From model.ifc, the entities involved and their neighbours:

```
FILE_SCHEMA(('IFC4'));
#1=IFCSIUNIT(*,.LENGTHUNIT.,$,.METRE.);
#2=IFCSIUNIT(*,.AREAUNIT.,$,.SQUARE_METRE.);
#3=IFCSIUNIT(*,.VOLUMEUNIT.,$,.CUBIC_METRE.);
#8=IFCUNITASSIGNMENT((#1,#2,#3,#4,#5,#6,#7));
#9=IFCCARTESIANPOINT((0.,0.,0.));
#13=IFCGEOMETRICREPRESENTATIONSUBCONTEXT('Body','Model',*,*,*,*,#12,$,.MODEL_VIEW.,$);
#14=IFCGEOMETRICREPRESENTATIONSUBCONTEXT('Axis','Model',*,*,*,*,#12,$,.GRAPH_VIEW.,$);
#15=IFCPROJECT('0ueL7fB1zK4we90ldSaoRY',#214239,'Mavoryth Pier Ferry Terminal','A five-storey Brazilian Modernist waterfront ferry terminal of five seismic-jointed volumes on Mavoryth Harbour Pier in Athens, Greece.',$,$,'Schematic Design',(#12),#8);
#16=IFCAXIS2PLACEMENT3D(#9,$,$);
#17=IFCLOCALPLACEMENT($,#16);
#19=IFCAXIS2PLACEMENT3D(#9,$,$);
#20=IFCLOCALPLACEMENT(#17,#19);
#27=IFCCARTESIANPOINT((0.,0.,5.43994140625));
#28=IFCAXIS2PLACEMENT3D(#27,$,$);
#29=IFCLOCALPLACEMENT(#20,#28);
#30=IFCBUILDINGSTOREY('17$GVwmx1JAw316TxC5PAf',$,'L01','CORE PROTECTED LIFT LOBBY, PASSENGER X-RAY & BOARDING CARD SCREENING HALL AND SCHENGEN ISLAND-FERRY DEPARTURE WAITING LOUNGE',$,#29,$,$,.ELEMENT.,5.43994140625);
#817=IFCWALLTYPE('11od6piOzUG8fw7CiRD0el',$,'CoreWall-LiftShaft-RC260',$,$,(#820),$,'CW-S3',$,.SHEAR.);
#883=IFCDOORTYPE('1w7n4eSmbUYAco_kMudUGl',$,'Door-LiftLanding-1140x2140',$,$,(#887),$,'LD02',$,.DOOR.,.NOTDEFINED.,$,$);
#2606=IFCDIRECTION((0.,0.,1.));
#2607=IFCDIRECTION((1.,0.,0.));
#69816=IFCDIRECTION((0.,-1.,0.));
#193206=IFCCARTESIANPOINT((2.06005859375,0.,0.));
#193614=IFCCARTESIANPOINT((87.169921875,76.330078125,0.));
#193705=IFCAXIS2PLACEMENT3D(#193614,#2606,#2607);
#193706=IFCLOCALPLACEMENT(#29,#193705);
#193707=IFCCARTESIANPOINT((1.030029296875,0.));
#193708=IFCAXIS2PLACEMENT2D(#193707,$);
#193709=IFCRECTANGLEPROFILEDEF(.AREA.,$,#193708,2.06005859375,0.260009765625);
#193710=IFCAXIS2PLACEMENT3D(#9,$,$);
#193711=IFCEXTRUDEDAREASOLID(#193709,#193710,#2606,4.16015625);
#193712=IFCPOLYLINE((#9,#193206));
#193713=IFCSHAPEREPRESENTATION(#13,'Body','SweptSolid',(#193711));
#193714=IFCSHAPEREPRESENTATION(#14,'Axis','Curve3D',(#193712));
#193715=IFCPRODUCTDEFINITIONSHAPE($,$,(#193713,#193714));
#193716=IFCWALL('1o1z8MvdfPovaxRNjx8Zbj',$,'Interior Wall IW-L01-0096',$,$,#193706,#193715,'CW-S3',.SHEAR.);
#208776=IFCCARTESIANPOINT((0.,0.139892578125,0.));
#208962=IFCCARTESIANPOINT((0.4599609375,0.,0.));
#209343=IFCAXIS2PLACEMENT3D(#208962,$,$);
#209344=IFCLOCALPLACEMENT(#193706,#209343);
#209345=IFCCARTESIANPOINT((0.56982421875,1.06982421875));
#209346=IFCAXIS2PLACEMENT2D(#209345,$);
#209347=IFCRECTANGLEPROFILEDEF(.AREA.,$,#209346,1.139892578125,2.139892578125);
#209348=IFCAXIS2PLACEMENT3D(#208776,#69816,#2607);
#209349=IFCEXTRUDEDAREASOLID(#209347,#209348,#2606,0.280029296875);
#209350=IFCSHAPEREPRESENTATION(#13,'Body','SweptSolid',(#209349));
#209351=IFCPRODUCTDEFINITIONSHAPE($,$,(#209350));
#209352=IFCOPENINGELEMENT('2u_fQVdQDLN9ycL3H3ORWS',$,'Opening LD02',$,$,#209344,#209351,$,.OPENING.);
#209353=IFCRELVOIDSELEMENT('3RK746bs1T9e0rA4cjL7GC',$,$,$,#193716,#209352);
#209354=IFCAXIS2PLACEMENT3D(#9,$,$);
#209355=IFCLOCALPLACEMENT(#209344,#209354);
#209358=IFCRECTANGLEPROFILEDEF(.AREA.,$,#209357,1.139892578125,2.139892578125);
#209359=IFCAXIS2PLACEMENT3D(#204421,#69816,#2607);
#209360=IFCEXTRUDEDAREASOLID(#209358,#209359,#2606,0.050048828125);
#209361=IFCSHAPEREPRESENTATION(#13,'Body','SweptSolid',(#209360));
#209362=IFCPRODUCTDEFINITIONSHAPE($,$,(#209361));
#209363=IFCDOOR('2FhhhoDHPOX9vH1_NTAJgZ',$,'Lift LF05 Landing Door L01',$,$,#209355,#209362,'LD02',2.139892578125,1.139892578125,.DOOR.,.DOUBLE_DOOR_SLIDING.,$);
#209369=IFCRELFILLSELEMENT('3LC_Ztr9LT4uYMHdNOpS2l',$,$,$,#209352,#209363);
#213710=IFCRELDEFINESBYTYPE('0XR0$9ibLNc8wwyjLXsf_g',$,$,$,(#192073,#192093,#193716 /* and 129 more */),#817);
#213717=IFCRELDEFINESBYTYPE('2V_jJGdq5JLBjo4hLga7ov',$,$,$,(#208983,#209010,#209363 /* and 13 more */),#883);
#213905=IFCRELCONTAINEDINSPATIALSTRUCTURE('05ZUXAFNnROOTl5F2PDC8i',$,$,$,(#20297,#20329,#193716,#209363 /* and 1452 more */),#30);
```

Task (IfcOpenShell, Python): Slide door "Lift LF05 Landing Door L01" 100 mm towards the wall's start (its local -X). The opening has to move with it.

```python
import ifcopenshell
import ifcopenshell.api.geometry
import ifcopenshell.util.placement
import ifcopenshell.util.unit

model = ifcopenshell.open("model.ifc")
unit_scale = ifcopenshell.util.unit.calculate_unit_scale(model)

door = model.by_id(209363)
opening = door.FillsVoids[0].RelatingOpeningElement
wall = opening.VoidsElements[0].RelatingBuildingElement

wall_matrix = ifcopenshell.util.placement.get_local_placement(wall.ObjectPlacement)
shift = wall_matrix[:3, 0] * -0.1 / unit_scale
before = ifcopenshell.util.placement.get_local_placement(door.ObjectPlacement)[:3, 3].copy()

# The door is placed relative to its opening, so it follows when the opening moves.
matrix = ifcopenshell.util.placement.get_local_placement(opening.ObjectPlacement)
matrix[:3, 3] += shift
ifcopenshell.api.geometry.edit_object_placement(
    model, product=opening, matrix=matrix, is_si=False, should_transform_children=True
)

after = ifcopenshell.util.placement.get_local_placement(door.ObjectPlacement)[:3, 3]
print("door moved by", (after - before).round(3) + 0.0)

model.write("model_edited.ifc")
```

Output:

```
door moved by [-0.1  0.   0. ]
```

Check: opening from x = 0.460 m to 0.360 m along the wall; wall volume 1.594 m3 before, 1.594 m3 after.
